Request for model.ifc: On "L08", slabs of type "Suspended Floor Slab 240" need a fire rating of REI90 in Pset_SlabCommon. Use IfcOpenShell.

First a look at what the model holds.

```python
import ifcopenshell
import ifcopenshell.util.element

model = ifcopenshell.open("model.ifc")
print(model.schema)
storey = next(s for s in model.by_type("IfcBuildingStorey") if s.Name == "L08")
slabs = [e for e in ifcopenshell.util.element.get_decomposition(storey) if e.is_a("IfcSlab")]
seen = {}
for e in slabs:
    element_type = ifcopenshell.util.element.get_type(e)
    key = (element_type.Name if element_type != e and element_type else None, ifcopenshell.util.element.get_pset(e, "Pset_SlabCommon", "FireRating"))
    seen[key] = seen.get(key, 0) + 1
for (name, value), count in sorted(seen.items(), key=str):
    print(count, "x", name, "|", value)
```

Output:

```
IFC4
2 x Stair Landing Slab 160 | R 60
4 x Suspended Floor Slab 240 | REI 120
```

```python
import ifcopenshell
import ifcopenshell.api.pset
import ifcopenshell.util.element

model = ifcopenshell.open("model.ifc")

storey = next(s for s in model.by_type("IfcBuildingStorey") if s.Name == "L08")
slabs = [e for e in ifcopenshell.util.element.get_decomposition(storey) if e.is_a("IfcSlab")]

count = 0
for e in slabs:
    element_type = ifcopenshell.util.element.get_type(e)
    if element_type in (None, e) or element_type.Name != "Suspended Floor Slab 240":
        continue
    # add_pset returns the element's existing set when there is one.
    pset = ifcopenshell.api.pset.add_pset(model, product=e, name="Pset_SlabCommon")
    ifcopenshell.api.pset.edit_pset(model, pset=pset, properties={"FireRating": "REI90"})
    count += 1

print(count, "slabs updated")

model.write("model_rev.ifc")
```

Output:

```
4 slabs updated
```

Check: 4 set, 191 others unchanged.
